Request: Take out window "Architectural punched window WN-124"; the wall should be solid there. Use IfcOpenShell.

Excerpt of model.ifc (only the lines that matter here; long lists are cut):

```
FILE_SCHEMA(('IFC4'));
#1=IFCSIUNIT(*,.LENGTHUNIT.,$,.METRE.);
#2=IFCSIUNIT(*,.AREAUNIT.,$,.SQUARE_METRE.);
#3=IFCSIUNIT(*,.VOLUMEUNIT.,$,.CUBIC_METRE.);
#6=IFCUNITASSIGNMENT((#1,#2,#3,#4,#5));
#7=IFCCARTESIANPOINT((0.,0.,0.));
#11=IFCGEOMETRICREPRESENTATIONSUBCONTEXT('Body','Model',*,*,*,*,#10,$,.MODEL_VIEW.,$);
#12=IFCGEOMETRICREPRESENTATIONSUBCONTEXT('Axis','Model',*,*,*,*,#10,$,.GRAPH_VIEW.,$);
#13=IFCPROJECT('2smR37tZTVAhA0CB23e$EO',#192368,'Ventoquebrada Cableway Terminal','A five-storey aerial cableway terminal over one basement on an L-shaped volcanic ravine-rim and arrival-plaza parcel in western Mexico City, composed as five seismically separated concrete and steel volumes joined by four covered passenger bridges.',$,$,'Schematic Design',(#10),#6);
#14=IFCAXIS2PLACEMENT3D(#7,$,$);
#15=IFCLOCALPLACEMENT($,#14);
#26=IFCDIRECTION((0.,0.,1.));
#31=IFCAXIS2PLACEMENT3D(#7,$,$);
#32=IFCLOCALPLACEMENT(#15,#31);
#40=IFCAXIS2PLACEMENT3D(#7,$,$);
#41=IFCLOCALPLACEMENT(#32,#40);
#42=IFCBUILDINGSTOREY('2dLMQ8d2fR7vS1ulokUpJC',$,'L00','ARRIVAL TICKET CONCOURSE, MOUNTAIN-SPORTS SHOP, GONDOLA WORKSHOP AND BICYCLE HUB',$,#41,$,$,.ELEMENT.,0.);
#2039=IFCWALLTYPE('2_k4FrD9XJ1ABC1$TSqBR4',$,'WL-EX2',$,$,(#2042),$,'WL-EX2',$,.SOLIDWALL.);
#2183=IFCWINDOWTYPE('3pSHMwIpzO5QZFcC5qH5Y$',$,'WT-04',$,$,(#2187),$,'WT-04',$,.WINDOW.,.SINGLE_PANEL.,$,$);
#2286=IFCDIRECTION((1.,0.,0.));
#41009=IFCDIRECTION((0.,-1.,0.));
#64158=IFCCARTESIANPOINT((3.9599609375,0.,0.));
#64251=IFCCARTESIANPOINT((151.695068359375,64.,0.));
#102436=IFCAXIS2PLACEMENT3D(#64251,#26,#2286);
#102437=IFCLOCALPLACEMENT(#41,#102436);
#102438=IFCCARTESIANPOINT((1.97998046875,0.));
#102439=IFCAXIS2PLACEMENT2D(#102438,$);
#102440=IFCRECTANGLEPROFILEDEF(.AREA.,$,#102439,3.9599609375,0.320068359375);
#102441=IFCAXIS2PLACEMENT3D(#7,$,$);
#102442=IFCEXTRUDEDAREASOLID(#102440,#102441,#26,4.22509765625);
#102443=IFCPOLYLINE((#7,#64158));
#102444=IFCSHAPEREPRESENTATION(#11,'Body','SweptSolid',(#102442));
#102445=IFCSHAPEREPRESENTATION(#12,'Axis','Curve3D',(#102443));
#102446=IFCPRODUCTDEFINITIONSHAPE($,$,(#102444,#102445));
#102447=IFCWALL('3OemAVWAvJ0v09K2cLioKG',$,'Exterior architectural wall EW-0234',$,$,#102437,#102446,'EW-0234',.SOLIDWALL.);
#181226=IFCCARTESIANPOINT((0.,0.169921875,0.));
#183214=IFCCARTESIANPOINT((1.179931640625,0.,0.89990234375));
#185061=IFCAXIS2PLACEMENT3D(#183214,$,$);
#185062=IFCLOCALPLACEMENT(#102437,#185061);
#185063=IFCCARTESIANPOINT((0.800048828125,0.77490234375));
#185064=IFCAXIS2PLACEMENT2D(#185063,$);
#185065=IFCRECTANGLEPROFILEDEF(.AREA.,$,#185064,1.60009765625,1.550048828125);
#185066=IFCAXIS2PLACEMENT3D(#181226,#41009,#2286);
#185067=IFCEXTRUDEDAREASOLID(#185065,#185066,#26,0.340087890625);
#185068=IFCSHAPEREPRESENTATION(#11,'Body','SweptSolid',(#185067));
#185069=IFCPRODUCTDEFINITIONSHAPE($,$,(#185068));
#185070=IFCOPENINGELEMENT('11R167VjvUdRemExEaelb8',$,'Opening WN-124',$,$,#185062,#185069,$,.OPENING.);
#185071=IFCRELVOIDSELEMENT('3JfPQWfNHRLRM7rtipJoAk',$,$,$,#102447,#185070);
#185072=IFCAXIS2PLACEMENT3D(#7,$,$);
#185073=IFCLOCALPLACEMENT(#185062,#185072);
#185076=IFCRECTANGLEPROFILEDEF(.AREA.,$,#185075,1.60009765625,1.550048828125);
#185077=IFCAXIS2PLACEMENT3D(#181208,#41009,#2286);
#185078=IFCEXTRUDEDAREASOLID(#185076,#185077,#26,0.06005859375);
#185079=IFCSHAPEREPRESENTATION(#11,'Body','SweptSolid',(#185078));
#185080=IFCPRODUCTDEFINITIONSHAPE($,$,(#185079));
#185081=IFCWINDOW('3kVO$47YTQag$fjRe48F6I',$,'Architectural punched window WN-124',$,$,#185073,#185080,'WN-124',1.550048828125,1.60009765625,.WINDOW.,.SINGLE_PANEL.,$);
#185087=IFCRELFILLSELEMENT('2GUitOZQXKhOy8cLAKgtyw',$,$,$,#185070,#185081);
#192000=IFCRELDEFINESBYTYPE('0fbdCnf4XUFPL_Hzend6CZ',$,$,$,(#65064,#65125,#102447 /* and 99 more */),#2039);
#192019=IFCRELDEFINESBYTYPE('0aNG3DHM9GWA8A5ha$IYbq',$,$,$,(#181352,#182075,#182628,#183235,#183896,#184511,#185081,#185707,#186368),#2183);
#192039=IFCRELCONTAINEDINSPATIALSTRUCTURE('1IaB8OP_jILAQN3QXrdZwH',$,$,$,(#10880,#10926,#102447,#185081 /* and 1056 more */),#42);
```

```python
import ifcopenshell
import ifcopenshell.api.feature
import ifcopenshell.api.root
import ifcopenshell.geom
import ifcopenshell.util.shape

model = ifcopenshell.open("model.ifc")
settings = ifcopenshell.geom.settings()


def volume(element):
    """Net volume in cubic metres, openings subtracted."""
    shape = ifcopenshell.geom.create_shape(settings, element)
    return ifcopenshell.util.shape.get_volume(shape.geometry)


window = model.by_guid("3kVO$47YTQag$fjRe48F6I")
opening = window.FillsVoids[0].RelatingOpeningElement
wall = opening.VoidsElements[0].RelatingBuildingElement
before = volume(wall)

ifcopenshell.api.root.remove_product(model, product=window)
ifcopenshell.api.feature.remove_feature(model, feature=opening)

after = volume(wall)

print(f"wall volume {before:.3f} -> {after:.3f} m3")

model.write("model-out.ifc")
```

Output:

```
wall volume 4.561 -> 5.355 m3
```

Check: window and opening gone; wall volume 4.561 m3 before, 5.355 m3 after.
